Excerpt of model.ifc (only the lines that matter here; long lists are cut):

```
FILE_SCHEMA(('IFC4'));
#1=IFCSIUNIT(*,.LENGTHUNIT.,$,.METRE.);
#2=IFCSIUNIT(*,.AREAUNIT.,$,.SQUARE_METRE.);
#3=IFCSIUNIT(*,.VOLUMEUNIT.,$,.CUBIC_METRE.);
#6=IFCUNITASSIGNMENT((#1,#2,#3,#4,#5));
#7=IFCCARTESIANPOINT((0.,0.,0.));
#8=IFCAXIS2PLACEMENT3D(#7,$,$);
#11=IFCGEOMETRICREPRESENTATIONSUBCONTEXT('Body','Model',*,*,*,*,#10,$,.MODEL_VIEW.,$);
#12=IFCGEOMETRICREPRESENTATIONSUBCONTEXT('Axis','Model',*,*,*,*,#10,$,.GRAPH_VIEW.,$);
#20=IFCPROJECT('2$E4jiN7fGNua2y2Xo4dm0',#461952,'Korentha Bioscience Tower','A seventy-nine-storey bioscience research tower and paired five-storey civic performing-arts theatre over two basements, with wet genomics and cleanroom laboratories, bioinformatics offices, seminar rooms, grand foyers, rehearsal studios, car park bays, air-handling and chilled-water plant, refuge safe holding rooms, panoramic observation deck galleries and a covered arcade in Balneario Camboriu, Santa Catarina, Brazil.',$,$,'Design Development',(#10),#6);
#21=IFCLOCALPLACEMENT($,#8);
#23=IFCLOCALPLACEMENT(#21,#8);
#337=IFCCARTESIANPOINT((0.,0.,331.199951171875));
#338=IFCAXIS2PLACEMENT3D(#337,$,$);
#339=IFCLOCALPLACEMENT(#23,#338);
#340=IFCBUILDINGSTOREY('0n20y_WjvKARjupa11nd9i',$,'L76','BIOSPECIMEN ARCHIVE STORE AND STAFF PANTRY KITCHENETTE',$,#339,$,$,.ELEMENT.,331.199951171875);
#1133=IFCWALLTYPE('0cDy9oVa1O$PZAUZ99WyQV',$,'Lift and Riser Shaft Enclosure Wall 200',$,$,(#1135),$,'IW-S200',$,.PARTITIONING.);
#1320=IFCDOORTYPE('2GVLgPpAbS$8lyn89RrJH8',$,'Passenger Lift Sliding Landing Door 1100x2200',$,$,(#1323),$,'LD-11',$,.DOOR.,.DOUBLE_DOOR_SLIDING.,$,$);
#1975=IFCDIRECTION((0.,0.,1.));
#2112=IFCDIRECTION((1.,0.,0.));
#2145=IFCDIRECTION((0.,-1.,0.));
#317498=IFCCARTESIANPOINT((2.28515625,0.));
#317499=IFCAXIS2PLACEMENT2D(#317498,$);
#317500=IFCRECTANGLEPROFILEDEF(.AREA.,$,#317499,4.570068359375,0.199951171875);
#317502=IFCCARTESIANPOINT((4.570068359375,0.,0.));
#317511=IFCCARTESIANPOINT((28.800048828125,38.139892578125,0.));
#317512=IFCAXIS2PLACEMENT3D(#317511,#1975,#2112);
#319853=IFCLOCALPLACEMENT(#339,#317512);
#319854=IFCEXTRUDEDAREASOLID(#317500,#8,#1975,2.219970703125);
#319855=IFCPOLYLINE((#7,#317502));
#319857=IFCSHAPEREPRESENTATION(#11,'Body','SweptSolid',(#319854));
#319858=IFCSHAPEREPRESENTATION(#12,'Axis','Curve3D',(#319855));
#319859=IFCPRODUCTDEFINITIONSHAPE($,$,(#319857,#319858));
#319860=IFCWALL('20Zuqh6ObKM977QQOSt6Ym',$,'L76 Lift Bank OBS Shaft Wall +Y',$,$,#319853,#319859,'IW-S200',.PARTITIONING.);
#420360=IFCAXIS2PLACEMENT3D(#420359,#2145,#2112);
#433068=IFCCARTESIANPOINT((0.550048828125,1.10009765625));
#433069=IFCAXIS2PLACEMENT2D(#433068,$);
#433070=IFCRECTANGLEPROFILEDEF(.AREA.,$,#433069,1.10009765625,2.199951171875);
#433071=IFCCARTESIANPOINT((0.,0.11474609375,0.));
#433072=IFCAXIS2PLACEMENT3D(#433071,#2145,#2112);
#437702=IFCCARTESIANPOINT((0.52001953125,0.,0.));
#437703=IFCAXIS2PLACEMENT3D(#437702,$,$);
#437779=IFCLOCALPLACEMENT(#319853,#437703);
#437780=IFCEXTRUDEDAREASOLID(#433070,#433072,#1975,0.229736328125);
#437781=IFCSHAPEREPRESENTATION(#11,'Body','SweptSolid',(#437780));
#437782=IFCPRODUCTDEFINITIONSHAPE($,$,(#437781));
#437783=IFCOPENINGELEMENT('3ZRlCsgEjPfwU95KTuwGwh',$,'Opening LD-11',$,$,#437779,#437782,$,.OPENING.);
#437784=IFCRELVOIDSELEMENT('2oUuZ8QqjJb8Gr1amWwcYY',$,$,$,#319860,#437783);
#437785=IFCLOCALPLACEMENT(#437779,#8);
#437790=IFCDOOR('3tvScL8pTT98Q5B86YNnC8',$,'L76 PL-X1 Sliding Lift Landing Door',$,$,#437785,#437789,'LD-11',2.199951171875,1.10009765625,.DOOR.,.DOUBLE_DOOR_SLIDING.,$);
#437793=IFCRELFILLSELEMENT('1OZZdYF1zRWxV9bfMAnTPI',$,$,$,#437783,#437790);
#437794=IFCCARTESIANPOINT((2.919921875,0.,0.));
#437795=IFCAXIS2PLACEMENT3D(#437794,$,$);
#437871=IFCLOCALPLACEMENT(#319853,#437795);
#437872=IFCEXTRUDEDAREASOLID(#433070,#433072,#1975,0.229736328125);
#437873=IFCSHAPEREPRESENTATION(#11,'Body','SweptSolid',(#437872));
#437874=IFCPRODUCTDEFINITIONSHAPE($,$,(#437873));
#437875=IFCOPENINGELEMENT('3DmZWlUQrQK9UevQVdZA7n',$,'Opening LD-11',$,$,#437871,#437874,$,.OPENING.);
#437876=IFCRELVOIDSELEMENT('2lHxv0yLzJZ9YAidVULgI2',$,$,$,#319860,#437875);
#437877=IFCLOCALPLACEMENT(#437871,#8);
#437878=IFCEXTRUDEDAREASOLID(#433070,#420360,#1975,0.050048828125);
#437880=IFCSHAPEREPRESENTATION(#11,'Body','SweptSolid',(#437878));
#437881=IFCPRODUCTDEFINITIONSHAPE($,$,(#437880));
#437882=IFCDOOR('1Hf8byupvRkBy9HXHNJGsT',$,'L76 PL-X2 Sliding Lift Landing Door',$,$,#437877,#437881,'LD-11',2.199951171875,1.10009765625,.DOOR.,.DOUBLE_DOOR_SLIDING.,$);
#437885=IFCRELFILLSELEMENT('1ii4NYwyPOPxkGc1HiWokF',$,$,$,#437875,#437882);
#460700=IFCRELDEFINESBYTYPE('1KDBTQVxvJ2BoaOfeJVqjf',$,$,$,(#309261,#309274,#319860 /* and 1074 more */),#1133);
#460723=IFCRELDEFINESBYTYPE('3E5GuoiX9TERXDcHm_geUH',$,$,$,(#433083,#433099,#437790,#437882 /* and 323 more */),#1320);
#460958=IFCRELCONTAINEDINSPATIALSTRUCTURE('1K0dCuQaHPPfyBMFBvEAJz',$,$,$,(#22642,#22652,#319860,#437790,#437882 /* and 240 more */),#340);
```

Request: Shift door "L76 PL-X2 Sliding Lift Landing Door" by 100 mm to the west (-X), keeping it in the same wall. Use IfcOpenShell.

```python
import ifcopenshell
import ifcopenshell.api.geometry
import ifcopenshell.util.placement

model = ifcopenshell.open("model.ifc")

door = model.by_guid("1Hf8byupvRkBy9HXHNJGsT")
opening = door.FillsVoids[0].RelatingOpeningElement
wall = opening.VoidsElements[0].RelatingBuildingElement

wall_matrix = ifcopenshell.util.placement.get_local_placement(wall.ObjectPlacement)
shift = wall_matrix[:3, 0] * -0.1
before = ifcopenshell.util.placement.get_local_placement(door.ObjectPlacement)[:3, 3].copy()

# The door is placed relative to its opening, so it follows when the opening moves.
matrix = ifcopenshell.util.placement.get_local_placement(opening.ObjectPlacement)
matrix[:3, 3] += shift
ifcopenshell.api.geometry.edit_object_placement(
    model, product=opening, matrix=matrix, is_si=False, should_transform_children=True
)

after = ifcopenshell.util.placement.get_local_placement(door.ObjectPlacement)[:3, 3]
print("door moved by", (after - before).round(3) + 0.0)

model.write("model-out.ifc")
```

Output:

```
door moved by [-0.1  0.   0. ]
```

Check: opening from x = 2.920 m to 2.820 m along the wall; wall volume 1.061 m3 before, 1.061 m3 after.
